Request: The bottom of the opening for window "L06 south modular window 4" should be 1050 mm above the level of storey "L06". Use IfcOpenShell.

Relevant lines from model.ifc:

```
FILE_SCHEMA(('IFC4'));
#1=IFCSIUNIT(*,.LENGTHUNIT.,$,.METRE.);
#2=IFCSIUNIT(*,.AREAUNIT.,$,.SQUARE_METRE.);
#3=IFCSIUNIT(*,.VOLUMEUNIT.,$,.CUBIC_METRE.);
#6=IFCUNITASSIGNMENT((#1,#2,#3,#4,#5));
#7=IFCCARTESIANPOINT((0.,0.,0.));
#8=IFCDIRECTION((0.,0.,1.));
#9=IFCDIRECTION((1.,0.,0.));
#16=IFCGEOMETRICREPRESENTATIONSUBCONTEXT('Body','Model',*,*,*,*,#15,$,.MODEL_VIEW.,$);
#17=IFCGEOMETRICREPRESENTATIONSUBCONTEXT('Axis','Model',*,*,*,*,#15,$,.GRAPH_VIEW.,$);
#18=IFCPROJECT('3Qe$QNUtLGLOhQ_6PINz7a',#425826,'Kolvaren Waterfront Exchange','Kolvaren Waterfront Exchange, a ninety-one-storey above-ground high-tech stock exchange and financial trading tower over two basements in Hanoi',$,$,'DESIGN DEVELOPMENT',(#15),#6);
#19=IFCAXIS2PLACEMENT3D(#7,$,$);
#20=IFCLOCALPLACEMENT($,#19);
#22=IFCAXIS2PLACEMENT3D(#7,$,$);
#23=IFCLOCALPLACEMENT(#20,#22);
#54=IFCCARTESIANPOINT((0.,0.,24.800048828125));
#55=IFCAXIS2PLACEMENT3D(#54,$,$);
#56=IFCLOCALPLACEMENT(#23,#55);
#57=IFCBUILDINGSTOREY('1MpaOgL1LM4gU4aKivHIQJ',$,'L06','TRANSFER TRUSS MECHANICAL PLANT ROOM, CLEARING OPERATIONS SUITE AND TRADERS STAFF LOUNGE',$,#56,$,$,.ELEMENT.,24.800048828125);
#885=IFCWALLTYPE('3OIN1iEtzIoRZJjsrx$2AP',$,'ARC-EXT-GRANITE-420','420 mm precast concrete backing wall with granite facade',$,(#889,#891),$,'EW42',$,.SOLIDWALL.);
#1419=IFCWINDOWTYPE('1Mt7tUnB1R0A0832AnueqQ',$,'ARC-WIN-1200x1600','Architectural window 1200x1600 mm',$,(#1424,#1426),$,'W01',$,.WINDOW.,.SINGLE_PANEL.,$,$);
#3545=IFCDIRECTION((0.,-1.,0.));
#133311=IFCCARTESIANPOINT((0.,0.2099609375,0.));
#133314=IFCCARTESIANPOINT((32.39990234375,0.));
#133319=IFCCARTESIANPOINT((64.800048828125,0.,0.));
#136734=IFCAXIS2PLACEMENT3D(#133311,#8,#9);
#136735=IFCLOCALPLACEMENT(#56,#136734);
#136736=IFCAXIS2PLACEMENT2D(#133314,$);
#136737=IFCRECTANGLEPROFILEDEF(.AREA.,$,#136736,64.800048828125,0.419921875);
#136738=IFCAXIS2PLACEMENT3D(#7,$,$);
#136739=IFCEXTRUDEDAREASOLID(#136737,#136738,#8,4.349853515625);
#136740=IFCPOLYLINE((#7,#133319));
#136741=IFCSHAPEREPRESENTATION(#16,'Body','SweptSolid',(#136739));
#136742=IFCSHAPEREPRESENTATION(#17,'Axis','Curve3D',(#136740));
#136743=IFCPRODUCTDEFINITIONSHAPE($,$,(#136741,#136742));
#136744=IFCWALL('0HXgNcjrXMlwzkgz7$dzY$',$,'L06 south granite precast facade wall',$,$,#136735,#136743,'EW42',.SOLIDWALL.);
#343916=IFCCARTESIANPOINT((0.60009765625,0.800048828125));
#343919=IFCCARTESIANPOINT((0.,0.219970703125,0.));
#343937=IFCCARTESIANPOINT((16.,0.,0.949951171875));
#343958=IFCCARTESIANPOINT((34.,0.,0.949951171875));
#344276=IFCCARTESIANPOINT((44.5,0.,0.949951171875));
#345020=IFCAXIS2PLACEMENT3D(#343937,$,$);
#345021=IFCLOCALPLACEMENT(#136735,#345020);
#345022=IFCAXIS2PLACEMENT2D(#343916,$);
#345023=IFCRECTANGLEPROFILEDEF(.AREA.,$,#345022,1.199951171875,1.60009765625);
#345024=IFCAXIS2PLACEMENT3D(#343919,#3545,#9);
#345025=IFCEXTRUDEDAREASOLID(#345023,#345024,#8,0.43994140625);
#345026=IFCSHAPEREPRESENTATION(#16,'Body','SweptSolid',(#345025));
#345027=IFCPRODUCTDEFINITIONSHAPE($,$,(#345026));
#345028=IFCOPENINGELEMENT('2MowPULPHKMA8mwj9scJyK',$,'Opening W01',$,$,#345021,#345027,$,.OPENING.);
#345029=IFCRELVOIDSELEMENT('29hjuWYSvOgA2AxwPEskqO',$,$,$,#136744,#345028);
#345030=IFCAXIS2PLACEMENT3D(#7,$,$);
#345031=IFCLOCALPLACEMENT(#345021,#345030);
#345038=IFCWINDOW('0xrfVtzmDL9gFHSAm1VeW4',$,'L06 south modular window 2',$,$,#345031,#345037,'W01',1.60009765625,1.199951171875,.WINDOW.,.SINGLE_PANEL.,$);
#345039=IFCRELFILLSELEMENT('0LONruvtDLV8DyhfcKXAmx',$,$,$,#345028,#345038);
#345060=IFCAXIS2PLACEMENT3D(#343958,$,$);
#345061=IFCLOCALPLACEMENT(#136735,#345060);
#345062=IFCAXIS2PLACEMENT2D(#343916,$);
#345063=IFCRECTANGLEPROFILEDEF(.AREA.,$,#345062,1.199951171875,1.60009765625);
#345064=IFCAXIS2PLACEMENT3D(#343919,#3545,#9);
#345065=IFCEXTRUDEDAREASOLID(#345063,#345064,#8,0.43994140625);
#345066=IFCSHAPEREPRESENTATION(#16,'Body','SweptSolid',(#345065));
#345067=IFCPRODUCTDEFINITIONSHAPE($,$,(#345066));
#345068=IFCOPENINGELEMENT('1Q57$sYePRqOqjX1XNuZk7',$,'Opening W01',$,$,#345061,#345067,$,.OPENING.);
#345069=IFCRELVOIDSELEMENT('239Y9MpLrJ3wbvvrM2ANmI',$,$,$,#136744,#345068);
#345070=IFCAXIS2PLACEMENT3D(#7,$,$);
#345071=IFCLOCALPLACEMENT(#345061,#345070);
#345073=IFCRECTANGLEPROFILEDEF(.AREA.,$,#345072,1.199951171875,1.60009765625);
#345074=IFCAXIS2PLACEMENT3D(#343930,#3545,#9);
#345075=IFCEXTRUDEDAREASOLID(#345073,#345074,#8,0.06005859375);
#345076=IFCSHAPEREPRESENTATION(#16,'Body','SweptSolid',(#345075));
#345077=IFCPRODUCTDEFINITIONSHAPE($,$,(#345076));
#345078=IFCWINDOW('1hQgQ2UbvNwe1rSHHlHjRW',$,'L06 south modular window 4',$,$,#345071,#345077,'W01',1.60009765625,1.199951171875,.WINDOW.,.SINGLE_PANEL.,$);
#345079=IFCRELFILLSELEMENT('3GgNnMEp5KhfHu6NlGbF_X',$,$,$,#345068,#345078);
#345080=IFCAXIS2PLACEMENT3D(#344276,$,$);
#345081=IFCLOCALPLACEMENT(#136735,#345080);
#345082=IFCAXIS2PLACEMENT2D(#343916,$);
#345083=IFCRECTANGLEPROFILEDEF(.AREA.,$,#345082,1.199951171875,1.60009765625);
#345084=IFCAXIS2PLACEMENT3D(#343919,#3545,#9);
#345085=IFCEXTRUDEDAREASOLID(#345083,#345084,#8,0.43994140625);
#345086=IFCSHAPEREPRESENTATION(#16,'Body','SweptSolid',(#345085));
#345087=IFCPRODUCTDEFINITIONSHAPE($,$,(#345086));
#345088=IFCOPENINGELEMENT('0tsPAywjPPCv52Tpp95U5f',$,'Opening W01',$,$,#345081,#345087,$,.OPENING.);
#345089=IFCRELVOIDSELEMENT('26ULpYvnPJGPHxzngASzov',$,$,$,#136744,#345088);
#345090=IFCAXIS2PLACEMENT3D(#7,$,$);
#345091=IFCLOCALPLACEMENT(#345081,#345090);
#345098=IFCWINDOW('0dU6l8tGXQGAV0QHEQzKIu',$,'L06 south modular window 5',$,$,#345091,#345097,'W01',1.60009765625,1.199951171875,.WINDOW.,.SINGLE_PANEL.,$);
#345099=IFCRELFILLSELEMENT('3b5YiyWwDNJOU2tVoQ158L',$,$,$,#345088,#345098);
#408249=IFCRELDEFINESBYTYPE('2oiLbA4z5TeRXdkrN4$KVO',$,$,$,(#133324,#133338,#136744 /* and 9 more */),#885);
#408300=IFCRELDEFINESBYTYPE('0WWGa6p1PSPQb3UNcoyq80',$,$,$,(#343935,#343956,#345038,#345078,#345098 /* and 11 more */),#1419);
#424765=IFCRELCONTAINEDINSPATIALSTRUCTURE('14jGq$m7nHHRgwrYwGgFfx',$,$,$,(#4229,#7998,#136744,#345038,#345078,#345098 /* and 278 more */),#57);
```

```python
import numpy as np
import ifcopenshell
import ifcopenshell.api.geometry
import ifcopenshell.geom
import ifcopenshell.util.element
import ifcopenshell.util.placement
import ifcopenshell.util.shape
import ifcopenshell.util.unit

model = ifcopenshell.open("model.ifc")
unit_scale = ifcopenshell.util.unit.calculate_unit_scale(model)

window = model.by_guid("1hQgQ2UbvNwe1rSHHlHjRW")
opening = window.FillsVoids[0].RelatingOpeningElement
storey = ifcopenshell.util.element.get_container(window, ifc_class="IfcBuildingStorey")
level = ifcopenshell.util.placement.get_local_placement(storey.ObjectPlacement)[2, 3]

# The opening's origin need not be at the sill, so measure its lowest point.
shape = ifcopenshell.geom.create_shape(ifcopenshell.geom.settings(), opening)
bottom = ifcopenshell.util.shape.get_shape_bottom_elevation(shape, shape.geometry) / unit_scale
dz = level + 1.05 / unit_scale - bottom

shift = np.array([0.0, 0.0, dz])
# The window is placed relative to its opening, so it follows when the opening moves.
matrix = ifcopenshell.util.placement.get_local_placement(opening.ObjectPlacement)
matrix[:3, 3] += shift
ifcopenshell.api.geometry.edit_object_placement(
    model, product=opening, matrix=matrix, is_si=False, should_transform_children=True
)

print(f"moved by {dz * unit_scale:+.3f} m")

model.write("model-out.ifc")
```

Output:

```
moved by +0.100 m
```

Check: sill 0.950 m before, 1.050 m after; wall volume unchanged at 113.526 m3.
